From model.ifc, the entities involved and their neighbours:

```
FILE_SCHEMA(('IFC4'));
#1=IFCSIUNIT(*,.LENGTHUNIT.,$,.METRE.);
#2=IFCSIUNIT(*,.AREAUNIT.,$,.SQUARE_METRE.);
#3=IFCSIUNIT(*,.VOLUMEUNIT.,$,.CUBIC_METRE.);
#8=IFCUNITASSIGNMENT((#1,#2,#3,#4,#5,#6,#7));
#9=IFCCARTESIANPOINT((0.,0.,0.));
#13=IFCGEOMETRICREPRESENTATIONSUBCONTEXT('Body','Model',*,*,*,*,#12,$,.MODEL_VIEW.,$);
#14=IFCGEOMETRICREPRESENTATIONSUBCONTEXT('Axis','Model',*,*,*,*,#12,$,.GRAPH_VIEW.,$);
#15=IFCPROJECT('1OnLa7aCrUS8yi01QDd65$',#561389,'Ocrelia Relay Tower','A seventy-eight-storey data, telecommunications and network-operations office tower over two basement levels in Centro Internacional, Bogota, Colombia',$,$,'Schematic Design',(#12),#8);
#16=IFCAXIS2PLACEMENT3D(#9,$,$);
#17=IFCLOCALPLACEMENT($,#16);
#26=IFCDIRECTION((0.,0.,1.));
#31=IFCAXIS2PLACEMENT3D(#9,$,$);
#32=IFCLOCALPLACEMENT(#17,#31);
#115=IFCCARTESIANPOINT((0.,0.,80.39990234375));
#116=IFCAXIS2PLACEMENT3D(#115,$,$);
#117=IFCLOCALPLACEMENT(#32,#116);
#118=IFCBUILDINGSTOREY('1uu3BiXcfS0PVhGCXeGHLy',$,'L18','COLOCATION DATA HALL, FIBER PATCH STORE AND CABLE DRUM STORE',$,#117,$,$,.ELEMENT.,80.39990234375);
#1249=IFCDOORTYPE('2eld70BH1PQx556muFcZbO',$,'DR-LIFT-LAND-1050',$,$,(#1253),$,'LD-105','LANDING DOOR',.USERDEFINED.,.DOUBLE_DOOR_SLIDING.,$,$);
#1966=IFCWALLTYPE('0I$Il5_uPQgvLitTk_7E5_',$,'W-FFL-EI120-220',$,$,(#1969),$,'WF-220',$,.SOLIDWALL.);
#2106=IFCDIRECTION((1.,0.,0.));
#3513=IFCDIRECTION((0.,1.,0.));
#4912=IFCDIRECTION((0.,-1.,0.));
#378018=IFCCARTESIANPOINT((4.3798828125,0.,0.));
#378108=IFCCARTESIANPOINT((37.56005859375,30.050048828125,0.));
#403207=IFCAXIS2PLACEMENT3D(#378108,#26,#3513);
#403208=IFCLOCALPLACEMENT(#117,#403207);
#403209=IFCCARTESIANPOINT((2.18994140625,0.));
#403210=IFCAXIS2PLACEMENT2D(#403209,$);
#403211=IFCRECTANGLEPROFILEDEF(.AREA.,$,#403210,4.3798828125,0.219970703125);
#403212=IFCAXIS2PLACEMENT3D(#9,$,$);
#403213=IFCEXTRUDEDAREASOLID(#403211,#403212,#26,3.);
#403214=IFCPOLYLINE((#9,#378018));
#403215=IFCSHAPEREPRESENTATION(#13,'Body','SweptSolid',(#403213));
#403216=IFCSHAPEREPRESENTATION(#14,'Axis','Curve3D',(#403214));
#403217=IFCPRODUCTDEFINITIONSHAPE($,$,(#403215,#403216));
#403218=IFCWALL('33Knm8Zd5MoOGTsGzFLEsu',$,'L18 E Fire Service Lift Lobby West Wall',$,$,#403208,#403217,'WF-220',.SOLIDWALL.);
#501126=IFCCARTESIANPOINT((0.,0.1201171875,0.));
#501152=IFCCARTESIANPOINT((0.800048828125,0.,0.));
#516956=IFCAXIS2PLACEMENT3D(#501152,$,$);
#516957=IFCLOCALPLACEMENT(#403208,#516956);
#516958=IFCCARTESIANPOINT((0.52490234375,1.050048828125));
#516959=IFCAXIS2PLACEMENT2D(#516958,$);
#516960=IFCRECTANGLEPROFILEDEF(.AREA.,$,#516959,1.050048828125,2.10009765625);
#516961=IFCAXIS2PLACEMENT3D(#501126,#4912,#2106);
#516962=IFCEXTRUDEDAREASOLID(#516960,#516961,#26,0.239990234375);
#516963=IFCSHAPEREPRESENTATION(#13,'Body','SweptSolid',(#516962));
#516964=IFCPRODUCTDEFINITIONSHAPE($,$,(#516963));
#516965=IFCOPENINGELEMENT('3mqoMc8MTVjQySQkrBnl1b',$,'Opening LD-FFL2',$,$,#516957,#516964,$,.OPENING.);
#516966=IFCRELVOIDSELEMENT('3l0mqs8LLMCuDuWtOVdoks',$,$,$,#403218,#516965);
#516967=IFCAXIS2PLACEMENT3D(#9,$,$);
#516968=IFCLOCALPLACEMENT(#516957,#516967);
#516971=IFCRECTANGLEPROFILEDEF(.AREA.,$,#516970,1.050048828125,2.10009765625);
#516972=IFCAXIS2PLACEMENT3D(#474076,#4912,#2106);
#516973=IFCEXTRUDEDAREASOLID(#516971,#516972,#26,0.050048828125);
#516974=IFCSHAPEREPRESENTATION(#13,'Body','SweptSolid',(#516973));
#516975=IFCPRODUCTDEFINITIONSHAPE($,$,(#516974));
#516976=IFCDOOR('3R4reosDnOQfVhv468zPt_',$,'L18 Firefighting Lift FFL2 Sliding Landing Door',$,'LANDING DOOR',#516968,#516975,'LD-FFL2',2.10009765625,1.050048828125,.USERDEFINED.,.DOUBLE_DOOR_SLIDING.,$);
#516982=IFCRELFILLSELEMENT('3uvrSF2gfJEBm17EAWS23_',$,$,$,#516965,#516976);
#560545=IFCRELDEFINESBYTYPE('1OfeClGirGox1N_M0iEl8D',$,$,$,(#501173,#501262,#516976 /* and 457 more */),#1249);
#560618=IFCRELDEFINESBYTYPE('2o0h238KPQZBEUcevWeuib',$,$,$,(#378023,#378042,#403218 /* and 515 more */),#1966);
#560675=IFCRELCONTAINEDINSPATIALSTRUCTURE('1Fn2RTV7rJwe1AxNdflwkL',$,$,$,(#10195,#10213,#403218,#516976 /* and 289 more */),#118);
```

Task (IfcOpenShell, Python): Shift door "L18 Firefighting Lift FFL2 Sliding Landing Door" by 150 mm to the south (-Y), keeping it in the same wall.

```python
import ifcopenshell
import ifcopenshell.api.geometry
import ifcopenshell.util.placement
import ifcopenshell.util.unit

model = ifcopenshell.open("model.ifc")
unit_scale = ifcopenshell.util.unit.calculate_unit_scale(model)

door = model.by_id(516976)
opening = door.FillsVoids[0].RelatingOpeningElement
wall = opening.VoidsElements[0].RelatingBuildingElement

wall_matrix = ifcopenshell.util.placement.get_local_placement(wall.ObjectPlacement)
shift = wall_matrix[:3, 0] * -0.15 / unit_scale
before = ifcopenshell.util.placement.get_local_placement(door.ObjectPlacement)[:3, 3].copy()

# The door is placed relative to its opening, so it follows when the opening moves.
matrix = ifcopenshell.util.placement.get_local_placement(opening.ObjectPlacement)
matrix[:3, 3] += shift
ifcopenshell.api.geometry.edit_object_placement(
    model, product=opening, matrix=matrix, is_si=False, should_transform_children=True
)

after = ifcopenshell.util.placement.get_local_placement(door.ObjectPlacement)[:3, 3]
print("door moved by", (after - before).round(3) + 0.0)

model.write("model_rev.ifc")
```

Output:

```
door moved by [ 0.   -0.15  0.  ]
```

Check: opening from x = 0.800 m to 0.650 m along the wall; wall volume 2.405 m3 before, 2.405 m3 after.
